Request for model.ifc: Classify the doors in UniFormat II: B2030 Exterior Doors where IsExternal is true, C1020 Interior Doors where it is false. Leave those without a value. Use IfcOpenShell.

First a look at what the model holds.

```python
import ifcopenshell
import ifcopenshell.util.element

model = ifcopenshell.open("model.ifc")
print(model.schema)
print("classifications:", [c.Name for c in model.by_type("IfcClassification")])
values = [ifcopenshell.util.element.get_pset(e, "Pset_DoorCommon", "IsExternal") for e in model.by_type("IfcDoor")]
for value in (True, False, None):
    print("IsExternal", value, values.count(value))
```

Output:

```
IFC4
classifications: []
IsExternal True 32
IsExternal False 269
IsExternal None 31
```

```python
import ifcopenshell
import ifcopenshell.api.classification
import ifcopenshell.util.element

model = ifcopenshell.open("model.ifc")

system = ifcopenshell.api.classification.add_classification(model, classification="UniFormat II")

doors = model.by_type("IfcDoor")
external = {e: ifcopenshell.util.element.get_pset(e, "Pset_DoorCommon", "IsExternal") for e in doors}
for flag, code, name in ((True, "B2030", "Exterior Doors"), (False, "C1020", "Interior Doors")):
    products = [e for e in doors if external[e] is flag]
    ifcopenshell.api.classification.add_reference(
        model, products=products, classification=system, identification=code, name=name
    )
    print(code, len(products))

model.write("model_edited.ifc")
```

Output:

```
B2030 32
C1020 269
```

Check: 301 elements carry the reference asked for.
